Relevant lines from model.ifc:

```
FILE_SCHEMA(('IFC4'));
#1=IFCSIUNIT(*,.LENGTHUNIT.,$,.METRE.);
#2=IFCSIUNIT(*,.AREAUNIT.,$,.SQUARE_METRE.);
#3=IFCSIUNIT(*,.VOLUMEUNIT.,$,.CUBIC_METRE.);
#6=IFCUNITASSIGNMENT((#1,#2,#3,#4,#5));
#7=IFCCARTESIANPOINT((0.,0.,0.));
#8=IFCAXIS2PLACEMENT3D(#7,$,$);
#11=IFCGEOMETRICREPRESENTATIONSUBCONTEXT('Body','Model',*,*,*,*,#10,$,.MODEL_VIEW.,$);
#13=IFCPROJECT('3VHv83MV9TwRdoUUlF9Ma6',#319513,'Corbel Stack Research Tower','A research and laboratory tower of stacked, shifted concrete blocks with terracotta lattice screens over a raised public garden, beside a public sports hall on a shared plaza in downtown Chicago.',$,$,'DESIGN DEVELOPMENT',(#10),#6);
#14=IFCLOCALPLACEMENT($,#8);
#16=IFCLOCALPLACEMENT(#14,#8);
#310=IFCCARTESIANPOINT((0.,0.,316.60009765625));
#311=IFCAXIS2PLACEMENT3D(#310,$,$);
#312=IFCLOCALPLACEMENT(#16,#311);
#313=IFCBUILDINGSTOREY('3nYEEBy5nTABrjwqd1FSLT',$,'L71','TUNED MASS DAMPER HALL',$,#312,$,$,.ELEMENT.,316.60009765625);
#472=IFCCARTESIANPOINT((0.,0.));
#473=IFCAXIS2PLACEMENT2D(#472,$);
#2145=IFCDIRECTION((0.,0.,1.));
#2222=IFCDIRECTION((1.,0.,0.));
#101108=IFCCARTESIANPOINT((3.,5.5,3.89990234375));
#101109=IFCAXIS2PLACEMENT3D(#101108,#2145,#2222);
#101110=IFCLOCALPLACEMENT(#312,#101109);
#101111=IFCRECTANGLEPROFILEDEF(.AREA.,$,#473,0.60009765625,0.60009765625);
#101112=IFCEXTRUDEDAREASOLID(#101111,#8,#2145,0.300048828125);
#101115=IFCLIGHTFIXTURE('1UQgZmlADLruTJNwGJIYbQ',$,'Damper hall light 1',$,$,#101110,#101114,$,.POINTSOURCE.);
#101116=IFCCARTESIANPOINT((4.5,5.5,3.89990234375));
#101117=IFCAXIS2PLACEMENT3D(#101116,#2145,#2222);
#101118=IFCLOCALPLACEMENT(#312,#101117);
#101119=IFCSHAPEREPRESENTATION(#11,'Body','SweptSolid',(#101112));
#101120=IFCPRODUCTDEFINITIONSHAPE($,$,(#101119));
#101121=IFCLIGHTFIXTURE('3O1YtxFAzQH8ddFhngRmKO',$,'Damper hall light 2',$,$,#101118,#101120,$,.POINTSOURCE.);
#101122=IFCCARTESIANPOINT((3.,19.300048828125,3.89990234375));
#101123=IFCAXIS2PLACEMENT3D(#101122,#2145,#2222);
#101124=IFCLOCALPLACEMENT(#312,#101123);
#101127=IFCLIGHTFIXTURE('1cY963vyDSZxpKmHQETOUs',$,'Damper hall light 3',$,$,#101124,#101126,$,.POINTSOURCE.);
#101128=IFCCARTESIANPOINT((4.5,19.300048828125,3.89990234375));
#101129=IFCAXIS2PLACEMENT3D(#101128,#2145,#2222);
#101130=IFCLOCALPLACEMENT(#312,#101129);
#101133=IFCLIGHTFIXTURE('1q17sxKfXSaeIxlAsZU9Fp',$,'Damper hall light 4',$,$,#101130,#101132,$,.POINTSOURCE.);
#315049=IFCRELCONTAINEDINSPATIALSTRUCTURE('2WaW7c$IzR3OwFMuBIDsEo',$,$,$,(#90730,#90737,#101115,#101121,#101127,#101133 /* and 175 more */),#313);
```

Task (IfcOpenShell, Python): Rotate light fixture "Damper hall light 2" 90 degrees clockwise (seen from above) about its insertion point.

```python
import ifcopenshell
import ifcopenshell.api.geometry
import ifcopenshell.util.placement

model = ifcopenshell.open("model.ifc")

item = model.by_guid("3O1YtxFAzQH8ddFhngRmKO")
matrix = ifcopenshell.util.placement.get_local_placement(item.ObjectPlacement)
matrix = matrix @ ifcopenshell.util.placement.rotation(-90, "Z")
ifcopenshell.api.geometry.edit_object_placement(model, product=item, matrix=matrix, is_si=False)

print(ifcopenshell.util.placement.get_local_placement(item.ObjectPlacement).round(3) + 0.0)

model.write("model-out.ifc")
```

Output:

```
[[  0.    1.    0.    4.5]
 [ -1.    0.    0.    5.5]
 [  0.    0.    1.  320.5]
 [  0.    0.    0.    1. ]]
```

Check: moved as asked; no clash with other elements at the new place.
